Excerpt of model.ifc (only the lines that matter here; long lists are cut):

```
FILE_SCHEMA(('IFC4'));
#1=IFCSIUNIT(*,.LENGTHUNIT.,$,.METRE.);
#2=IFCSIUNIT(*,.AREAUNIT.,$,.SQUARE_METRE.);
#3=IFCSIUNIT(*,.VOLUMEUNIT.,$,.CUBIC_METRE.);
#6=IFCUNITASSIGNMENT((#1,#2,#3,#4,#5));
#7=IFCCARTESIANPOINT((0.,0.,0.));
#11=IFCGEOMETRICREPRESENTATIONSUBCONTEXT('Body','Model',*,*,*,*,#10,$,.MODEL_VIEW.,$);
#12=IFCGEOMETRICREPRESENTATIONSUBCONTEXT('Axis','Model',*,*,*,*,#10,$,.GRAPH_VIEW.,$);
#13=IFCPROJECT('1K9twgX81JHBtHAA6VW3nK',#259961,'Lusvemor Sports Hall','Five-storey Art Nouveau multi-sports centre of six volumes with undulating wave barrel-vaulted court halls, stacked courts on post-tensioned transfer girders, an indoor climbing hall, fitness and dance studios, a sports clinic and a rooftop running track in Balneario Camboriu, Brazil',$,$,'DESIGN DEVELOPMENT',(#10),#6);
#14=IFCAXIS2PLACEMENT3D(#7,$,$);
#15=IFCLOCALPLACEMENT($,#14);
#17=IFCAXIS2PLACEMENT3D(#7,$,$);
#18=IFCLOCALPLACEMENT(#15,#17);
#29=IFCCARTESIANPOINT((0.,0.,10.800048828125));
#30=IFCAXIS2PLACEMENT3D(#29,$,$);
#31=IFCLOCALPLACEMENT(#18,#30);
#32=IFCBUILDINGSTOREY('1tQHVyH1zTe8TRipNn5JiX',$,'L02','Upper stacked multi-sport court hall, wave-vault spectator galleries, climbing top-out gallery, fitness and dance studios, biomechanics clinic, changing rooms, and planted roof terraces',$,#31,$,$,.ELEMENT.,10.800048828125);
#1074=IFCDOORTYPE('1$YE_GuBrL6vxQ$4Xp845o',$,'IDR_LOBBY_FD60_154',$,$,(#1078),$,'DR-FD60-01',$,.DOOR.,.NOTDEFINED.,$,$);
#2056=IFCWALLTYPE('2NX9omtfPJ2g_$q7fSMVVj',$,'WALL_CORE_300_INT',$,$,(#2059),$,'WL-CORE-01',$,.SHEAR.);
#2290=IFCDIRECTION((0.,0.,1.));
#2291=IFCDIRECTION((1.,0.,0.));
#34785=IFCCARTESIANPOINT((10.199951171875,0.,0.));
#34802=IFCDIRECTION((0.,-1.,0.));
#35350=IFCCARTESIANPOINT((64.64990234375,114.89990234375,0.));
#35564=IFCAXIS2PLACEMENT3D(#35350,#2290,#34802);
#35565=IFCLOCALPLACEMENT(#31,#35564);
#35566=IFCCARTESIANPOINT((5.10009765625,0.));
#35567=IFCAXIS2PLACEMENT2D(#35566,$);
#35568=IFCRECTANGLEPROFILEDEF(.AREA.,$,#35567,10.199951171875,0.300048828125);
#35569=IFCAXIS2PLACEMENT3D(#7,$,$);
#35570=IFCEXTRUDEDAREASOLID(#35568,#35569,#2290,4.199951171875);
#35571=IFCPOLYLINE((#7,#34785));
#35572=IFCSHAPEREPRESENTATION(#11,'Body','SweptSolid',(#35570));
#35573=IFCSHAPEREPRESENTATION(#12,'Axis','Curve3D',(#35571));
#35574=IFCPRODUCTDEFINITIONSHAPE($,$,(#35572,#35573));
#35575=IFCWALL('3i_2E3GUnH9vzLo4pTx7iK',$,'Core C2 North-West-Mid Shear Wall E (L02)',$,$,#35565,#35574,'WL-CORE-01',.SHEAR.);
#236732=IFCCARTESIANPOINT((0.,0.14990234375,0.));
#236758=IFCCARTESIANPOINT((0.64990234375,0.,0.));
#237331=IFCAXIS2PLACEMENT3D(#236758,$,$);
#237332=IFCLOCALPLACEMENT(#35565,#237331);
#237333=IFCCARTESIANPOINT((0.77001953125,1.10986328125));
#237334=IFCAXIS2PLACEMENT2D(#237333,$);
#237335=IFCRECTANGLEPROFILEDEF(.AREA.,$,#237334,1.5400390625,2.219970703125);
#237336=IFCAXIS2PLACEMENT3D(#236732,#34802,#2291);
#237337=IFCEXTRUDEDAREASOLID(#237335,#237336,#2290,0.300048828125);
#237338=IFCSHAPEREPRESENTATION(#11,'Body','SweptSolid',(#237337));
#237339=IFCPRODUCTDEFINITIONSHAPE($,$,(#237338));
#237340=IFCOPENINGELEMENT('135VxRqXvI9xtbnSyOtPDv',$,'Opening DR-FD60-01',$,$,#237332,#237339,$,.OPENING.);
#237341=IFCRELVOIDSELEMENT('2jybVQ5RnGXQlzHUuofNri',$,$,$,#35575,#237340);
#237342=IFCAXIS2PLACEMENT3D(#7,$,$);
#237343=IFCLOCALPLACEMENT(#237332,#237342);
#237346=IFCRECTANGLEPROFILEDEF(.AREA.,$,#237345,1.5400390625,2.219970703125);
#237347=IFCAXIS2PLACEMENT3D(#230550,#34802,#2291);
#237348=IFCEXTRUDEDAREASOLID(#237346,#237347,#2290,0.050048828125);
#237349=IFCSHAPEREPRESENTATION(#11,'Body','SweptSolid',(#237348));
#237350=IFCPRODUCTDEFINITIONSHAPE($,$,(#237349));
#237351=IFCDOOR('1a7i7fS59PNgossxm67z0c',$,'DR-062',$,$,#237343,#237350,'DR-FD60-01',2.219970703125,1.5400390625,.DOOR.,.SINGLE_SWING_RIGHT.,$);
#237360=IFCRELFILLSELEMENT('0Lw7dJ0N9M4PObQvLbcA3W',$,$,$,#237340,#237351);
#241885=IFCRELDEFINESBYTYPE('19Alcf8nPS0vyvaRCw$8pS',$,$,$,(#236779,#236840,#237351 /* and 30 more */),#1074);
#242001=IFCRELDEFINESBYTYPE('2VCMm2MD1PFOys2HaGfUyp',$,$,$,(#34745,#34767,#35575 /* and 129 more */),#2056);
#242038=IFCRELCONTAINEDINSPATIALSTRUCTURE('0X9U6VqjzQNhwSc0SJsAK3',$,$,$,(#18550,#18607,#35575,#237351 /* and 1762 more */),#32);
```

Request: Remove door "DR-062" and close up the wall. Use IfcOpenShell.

```python
import ifcopenshell
import ifcopenshell.api.feature
import ifcopenshell.api.root
import ifcopenshell.geom
import ifcopenshell.util.shape

model = ifcopenshell.open("model.ifc")
settings = ifcopenshell.geom.settings()


def volume(element):
    """Net volume in cubic metres, openings subtracted."""
    shape = ifcopenshell.geom.create_shape(settings, element)
    return ifcopenshell.util.shape.get_volume(shape.geometry)


door = model.by_guid("1a7i7fS59PNgossxm67z0c")
opening = door.FillsVoids[0].RelatingOpeningElement
wall = opening.VoidsElements[0].RelatingBuildingElement
before = volume(wall)

ifcopenshell.api.root.remove_product(model, product=door)
ifcopenshell.api.feature.remove_feature(model, feature=opening)

after = volume(wall)

print(f"wall volume {before:.3f} -> {after:.3f} m3")

model.write("model_v2.ifc")
```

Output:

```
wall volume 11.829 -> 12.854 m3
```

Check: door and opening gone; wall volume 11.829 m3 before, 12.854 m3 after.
